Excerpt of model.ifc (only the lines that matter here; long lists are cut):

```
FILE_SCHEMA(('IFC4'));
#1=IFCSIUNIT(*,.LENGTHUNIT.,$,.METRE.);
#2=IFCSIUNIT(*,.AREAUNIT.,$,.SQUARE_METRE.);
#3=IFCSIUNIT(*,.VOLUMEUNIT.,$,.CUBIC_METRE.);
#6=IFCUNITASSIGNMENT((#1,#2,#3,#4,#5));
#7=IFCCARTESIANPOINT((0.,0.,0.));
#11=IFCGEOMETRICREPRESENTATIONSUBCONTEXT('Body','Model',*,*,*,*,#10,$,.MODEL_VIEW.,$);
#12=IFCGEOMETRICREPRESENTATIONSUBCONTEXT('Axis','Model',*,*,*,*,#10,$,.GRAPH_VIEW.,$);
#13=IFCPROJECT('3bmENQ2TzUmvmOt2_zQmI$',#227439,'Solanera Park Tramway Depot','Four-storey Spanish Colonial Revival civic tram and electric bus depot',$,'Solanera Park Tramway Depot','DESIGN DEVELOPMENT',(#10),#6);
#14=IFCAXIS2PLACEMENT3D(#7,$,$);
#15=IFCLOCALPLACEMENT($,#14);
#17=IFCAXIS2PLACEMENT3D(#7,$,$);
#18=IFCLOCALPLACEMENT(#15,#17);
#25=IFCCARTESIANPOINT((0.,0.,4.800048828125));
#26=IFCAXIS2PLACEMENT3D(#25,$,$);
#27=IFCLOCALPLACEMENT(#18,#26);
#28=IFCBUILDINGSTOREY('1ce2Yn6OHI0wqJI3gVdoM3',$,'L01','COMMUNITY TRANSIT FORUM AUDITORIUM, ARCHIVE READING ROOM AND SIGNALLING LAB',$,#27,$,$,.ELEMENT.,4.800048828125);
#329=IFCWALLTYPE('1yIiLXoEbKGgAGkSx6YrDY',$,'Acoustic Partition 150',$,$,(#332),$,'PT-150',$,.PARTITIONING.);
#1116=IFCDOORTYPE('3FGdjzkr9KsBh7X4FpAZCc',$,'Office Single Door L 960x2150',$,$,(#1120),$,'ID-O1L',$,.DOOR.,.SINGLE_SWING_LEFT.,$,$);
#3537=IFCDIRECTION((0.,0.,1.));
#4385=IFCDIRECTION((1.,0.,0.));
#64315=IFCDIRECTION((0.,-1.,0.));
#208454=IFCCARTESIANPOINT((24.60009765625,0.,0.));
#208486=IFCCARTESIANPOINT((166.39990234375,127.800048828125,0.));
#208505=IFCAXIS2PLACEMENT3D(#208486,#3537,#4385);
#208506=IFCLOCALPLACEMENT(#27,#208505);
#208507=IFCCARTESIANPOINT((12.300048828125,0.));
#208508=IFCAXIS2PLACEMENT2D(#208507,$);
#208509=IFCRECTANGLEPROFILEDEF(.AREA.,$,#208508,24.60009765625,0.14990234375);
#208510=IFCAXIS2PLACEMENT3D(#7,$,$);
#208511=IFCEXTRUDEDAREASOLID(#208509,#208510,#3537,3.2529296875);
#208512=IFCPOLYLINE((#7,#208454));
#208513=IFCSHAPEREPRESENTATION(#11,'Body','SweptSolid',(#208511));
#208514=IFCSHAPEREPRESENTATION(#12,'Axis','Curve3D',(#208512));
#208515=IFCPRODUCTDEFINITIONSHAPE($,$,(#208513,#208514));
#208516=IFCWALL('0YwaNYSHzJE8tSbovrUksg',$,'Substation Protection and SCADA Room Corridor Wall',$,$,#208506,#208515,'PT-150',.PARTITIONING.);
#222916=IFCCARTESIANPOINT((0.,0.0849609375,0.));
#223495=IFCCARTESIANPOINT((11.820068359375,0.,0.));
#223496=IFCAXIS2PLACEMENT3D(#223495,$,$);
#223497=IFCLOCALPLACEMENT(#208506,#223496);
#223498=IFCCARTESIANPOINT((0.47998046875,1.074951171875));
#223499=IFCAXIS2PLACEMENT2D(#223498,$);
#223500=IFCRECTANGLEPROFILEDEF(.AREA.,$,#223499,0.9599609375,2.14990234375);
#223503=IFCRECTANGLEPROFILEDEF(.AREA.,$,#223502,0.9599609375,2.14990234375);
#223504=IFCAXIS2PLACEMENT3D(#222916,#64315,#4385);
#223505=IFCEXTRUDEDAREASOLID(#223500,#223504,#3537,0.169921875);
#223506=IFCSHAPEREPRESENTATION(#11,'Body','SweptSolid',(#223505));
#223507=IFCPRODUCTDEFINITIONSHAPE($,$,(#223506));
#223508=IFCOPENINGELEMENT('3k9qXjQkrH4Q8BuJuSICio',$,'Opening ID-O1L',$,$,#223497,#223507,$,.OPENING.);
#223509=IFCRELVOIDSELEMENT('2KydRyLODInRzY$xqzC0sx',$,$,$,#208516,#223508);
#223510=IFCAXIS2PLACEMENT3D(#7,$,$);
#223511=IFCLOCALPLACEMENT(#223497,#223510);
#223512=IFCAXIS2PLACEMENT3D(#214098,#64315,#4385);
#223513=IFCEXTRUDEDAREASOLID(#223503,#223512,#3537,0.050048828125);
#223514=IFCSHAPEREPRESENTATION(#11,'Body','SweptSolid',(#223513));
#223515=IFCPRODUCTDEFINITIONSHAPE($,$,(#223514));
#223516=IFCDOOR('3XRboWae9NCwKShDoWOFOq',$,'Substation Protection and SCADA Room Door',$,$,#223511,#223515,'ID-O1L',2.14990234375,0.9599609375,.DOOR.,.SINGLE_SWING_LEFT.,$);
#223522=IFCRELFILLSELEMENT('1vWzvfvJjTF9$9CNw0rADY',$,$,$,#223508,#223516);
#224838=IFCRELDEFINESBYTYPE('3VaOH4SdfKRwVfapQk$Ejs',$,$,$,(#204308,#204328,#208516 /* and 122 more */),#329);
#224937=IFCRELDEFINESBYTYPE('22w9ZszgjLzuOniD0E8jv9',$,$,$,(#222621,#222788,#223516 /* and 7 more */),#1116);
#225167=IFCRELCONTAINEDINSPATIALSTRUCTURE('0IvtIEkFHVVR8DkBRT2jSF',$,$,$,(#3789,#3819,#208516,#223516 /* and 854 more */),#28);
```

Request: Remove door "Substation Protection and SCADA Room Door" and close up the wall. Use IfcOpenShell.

```python
import ifcopenshell
import ifcopenshell.api.feature
import ifcopenshell.api.root
import ifcopenshell.geom
import ifcopenshell.util.shape

model = ifcopenshell.open("model.ifc")
settings = ifcopenshell.geom.settings()


def volume(element):
    """Net volume in cubic metres, openings subtracted."""
    shape = ifcopenshell.geom.create_shape(settings, element)
    return ifcopenshell.util.shape.get_volume(shape.geometry)


door = model.by_guid("3XRboWae9NCwKShDoWOFOq")
opening = door.FillsVoids[0].RelatingOpeningElement
wall = opening.VoidsElements[0].RelatingBuildingElement
before = volume(wall)

ifcopenshell.api.root.remove_product(model, product=door)
ifcopenshell.api.feature.remove_feature(model, feature=opening)

after = volume(wall)

print(f"wall volume {before:.3f} -> {after:.3f} m3")

model.write("model_edited.ifc")
```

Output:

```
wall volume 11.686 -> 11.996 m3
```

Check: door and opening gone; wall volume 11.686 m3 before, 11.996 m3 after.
